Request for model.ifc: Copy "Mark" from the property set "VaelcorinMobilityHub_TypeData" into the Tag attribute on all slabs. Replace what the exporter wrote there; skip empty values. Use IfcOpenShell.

First a look at what the model holds.

```python
import ifcopenshell
import ifcopenshell.util.element

model = ifcopenshell.open("model.ifc")
print(model.schema)
slabs = model.by_type("IfcSlab")
print(len(slabs), "slabs")
for e in slabs[:8]:
    source = ifcopenshell.util.element.get_pset(e, "VaelcorinMobilityHub_TypeData", "Mark")
    target = e.Tag
    print(e.id(), repr(source), repr(target), sep=" | ")
```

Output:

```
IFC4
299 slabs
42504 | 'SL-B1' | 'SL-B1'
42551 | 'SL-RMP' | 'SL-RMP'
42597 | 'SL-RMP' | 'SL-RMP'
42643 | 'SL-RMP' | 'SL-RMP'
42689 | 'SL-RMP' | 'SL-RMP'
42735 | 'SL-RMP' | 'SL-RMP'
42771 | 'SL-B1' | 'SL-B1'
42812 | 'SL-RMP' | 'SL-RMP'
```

```python
import ifcopenshell
import ifcopenshell.util.element

model = ifcopenshell.open("model.ifc")

count = 0
for e in model.by_type("IfcSlab"):
    value = ifcopenshell.util.element.get_pset(e, "VaelcorinMobilityHub_TypeData", "Mark")
    current = e.Tag
    if not value or not value.strip() or current == value:
        continue
    e.Tag = value
    count += 1

print(count, "slabs updated")

model.write("model_edited.ifc")
```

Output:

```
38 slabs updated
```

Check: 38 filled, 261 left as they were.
